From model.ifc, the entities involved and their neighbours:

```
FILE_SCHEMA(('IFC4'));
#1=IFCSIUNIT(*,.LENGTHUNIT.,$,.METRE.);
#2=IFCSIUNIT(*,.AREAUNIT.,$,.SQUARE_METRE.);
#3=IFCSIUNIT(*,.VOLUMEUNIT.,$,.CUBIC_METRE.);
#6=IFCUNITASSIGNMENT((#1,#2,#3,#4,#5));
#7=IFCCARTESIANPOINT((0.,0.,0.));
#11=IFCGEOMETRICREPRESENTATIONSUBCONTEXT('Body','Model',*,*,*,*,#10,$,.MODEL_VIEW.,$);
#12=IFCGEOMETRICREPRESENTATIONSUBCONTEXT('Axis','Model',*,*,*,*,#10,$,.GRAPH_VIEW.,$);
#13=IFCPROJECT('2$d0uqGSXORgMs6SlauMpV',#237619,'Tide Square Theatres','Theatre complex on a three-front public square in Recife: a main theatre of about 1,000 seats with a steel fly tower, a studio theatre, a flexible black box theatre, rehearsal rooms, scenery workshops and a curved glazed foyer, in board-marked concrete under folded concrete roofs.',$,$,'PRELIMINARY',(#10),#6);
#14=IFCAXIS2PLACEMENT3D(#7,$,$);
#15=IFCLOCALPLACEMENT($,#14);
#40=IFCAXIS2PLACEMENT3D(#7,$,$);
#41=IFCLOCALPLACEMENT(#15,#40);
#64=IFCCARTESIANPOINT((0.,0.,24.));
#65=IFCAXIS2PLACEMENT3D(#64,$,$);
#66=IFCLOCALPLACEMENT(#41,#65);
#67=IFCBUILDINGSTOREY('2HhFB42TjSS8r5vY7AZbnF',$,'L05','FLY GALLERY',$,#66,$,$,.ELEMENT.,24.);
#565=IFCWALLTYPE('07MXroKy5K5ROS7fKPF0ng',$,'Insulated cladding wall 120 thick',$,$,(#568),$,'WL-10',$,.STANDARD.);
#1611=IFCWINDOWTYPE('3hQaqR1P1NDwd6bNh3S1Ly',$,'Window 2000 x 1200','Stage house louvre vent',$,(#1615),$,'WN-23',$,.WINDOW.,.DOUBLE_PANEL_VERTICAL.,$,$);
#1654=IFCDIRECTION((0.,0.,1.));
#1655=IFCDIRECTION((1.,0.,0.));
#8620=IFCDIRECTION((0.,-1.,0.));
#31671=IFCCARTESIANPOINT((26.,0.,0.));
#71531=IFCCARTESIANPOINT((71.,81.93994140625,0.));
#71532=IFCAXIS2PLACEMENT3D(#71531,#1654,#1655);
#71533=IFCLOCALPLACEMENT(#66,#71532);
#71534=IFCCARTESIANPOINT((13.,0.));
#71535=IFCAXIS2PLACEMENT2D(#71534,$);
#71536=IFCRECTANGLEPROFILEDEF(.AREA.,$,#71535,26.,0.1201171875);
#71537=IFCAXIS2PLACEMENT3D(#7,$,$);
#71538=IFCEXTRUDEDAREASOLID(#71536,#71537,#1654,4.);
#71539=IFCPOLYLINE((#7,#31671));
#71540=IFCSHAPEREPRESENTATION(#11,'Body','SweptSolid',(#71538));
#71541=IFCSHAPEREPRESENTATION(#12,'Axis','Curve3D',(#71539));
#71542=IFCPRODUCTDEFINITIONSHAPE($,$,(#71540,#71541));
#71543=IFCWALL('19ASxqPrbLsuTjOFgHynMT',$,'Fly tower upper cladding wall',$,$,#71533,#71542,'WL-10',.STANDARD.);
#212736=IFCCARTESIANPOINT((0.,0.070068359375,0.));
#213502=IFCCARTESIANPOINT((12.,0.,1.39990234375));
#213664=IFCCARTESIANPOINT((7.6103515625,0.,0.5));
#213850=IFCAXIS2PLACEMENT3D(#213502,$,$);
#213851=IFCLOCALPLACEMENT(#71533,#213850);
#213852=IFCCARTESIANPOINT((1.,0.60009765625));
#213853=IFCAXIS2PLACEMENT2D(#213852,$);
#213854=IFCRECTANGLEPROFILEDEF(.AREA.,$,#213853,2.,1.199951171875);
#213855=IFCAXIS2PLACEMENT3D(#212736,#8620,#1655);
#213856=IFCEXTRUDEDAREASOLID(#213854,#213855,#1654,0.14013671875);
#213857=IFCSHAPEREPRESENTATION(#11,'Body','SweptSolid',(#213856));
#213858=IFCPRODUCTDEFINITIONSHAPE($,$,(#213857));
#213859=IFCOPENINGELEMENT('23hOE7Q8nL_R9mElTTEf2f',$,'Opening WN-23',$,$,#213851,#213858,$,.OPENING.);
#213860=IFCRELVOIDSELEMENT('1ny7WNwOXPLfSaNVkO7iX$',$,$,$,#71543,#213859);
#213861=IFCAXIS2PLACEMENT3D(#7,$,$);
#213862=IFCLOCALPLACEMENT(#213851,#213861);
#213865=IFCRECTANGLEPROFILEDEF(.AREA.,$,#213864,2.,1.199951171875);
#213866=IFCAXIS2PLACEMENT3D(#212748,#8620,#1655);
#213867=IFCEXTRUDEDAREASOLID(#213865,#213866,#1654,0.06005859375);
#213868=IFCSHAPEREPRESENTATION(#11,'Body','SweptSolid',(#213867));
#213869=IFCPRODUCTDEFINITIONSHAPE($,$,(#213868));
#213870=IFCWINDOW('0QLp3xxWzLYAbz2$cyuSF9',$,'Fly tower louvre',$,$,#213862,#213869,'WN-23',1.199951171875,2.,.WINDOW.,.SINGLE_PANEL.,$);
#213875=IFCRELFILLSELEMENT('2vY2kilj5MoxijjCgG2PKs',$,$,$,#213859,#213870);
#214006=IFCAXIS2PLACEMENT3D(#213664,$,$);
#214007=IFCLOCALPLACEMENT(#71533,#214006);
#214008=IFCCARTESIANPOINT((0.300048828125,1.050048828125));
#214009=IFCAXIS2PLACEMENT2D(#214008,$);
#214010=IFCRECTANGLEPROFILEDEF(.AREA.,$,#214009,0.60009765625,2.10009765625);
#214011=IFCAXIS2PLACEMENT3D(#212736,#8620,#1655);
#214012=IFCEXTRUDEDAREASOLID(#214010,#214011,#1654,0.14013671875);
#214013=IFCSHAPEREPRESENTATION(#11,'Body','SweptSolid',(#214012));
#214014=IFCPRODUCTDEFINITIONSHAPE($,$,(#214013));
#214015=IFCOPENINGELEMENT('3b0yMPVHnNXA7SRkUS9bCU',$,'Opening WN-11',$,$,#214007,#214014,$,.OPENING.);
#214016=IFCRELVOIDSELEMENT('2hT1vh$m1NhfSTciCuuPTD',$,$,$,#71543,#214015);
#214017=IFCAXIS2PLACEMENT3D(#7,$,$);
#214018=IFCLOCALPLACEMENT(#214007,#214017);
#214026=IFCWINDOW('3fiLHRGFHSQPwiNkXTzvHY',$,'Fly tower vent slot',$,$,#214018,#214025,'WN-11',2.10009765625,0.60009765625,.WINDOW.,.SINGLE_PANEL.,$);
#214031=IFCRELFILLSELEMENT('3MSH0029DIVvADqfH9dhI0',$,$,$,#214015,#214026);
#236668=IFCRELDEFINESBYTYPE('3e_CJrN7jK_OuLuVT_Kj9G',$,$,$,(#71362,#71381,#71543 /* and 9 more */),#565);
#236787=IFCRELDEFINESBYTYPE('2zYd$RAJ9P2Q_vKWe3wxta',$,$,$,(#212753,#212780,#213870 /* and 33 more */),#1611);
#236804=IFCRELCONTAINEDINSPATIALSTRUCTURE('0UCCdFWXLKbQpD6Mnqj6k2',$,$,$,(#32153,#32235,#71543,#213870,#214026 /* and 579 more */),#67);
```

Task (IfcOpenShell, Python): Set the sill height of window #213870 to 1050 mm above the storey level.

```python
import numpy as np
import ifcopenshell
import ifcopenshell.api.geometry
import ifcopenshell.geom
import ifcopenshell.util.element
import ifcopenshell.util.placement
import ifcopenshell.util.shape
import ifcopenshell.util.unit

model = ifcopenshell.open("model.ifc")
unit_scale = ifcopenshell.util.unit.calculate_unit_scale(model)

window = model.by_guid("0QLp3xxWzLYAbz2$cyuSF9")
opening = window.FillsVoids[0].RelatingOpeningElement
storey = ifcopenshell.util.element.get_container(window, ifc_class="IfcBuildingStorey")
level = ifcopenshell.util.placement.get_local_placement(storey.ObjectPlacement)[2, 3]

# The opening's origin need not be at the sill, so measure its lowest point.
shape = ifcopenshell.geom.create_shape(ifcopenshell.geom.settings(), opening)
bottom = ifcopenshell.util.shape.get_shape_bottom_elevation(shape, shape.geometry) / unit_scale
dz = level + 1.05 - bottom

shift = np.array([0.0, 0.0, dz])
# The window is placed relative to its opening, so it follows when the opening moves.
matrix = ifcopenshell.util.placement.get_local_placement(opening.ObjectPlacement)
matrix[:3, 3] += shift
ifcopenshell.api.geometry.edit_object_placement(
    model, product=opening, matrix=matrix, is_si=False, should_transform_children=True
)

print(f"moved by {dz * unit_scale:+.3f} m")

model.write("model_edited.ifc")
```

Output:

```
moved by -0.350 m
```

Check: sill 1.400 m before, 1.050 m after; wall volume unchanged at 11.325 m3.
